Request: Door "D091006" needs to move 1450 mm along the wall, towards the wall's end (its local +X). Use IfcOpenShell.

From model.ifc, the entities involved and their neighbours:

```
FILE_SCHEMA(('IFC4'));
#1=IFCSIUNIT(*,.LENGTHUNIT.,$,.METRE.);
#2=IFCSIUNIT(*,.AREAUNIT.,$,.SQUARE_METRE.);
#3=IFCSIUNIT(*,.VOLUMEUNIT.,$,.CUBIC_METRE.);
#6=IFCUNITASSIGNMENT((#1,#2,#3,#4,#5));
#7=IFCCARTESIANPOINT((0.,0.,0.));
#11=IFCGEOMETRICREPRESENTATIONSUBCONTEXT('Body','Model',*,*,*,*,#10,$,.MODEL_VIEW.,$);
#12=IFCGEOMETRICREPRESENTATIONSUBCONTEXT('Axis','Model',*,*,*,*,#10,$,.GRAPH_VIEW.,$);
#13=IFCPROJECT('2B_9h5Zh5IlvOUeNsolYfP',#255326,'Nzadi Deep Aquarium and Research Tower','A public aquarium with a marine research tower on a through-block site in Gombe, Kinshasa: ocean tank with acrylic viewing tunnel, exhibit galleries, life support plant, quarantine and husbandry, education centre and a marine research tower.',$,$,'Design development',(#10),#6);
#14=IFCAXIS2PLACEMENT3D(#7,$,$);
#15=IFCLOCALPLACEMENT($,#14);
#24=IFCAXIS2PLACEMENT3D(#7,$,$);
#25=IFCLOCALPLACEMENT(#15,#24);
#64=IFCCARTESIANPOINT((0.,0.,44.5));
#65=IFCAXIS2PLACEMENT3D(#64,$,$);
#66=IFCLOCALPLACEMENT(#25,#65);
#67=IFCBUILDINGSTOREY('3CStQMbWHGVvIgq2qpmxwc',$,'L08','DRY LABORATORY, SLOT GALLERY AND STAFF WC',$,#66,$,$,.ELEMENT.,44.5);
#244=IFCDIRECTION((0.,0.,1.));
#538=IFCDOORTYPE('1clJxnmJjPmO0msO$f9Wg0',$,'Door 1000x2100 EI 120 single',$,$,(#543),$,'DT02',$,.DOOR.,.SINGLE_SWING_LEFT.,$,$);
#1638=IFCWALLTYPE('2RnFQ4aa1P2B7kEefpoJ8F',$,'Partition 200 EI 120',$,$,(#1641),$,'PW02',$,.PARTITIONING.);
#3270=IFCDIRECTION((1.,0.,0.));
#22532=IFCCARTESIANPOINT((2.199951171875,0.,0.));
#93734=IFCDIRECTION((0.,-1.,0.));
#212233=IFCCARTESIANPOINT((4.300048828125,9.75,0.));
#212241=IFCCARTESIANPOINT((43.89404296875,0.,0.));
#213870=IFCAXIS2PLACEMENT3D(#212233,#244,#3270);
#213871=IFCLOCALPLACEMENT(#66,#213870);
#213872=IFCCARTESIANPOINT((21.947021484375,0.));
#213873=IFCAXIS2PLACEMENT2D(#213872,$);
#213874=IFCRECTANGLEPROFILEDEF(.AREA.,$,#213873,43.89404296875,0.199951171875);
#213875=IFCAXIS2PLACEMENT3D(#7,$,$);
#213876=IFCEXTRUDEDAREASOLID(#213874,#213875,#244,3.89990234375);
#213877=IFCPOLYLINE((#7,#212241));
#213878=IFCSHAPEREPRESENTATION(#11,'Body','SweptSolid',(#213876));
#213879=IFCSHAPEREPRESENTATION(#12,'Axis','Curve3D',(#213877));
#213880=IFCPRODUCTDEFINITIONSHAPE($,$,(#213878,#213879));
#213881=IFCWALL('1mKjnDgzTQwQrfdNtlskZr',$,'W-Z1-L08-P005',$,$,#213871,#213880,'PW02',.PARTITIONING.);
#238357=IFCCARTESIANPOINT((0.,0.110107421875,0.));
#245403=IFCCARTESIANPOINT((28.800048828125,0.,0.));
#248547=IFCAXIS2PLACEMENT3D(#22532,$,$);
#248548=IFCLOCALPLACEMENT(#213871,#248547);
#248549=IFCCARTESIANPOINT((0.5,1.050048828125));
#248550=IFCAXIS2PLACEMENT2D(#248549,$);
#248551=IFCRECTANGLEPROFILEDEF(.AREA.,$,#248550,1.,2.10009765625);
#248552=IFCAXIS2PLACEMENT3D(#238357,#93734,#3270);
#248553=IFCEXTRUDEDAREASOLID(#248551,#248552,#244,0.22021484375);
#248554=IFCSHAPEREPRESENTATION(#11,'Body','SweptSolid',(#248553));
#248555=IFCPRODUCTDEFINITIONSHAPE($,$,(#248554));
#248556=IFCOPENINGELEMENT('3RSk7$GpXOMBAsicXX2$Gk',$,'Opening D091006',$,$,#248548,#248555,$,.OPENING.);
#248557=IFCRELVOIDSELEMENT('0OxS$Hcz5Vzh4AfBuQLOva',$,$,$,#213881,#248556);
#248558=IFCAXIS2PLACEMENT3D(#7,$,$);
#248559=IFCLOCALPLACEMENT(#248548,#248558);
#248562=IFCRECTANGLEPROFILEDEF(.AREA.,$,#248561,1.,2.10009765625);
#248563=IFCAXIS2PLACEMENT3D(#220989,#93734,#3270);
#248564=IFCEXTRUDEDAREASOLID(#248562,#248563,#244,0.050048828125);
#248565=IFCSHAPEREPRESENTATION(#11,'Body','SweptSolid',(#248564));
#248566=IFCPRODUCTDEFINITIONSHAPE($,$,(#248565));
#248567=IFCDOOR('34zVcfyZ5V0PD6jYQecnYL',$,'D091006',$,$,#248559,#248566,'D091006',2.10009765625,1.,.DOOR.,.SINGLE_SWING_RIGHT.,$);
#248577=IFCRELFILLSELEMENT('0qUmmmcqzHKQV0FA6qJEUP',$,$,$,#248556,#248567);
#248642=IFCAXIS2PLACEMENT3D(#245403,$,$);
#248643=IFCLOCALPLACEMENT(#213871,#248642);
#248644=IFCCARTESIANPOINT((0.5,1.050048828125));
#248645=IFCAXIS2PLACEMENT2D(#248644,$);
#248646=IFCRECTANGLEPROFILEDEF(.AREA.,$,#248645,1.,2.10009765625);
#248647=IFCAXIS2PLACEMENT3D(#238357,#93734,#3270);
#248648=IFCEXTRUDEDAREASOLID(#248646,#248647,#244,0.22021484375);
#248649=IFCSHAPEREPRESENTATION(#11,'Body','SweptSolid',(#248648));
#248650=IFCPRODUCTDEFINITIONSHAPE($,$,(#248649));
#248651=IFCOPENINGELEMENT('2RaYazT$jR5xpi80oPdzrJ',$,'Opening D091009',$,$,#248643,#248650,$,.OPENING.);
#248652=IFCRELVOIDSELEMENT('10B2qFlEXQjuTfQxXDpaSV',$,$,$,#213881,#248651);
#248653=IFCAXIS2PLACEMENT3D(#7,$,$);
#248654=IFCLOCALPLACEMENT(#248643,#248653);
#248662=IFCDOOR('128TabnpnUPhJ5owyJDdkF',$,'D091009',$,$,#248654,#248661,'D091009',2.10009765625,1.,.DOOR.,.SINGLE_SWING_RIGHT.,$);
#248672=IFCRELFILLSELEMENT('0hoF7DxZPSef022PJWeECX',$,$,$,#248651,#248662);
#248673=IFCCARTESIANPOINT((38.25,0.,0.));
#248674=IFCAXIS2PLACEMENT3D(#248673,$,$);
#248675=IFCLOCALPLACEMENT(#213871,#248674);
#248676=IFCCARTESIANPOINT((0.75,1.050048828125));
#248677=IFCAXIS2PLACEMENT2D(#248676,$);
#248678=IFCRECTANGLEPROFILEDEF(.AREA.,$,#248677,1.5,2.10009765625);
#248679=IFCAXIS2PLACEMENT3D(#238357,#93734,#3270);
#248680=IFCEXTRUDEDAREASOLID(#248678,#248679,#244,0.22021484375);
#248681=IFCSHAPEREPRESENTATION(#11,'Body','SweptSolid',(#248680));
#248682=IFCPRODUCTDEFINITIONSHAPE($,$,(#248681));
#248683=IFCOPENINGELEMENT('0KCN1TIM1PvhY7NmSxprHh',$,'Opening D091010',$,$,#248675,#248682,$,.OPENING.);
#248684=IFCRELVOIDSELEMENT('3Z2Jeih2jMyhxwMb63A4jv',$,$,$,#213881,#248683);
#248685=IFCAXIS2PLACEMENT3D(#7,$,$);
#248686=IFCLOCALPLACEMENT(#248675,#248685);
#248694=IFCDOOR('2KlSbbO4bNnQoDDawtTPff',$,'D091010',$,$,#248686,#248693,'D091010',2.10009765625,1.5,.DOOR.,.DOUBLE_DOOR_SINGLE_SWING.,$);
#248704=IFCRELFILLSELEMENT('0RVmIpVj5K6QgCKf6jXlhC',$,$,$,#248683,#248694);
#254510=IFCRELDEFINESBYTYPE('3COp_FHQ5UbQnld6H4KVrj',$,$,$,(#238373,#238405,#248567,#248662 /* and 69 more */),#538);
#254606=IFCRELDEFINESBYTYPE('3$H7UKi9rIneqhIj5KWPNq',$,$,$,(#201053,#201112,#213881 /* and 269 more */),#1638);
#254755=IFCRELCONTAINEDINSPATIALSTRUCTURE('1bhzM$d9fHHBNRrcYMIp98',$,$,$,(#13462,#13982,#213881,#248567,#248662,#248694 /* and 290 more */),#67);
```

```python
import ifcopenshell
import ifcopenshell.api.geometry
import ifcopenshell.util.placement
import ifcopenshell.util.unit

model = ifcopenshell.open("model.ifc")
unit_scale = ifcopenshell.util.unit.calculate_unit_scale(model)

door = model.by_guid("34zVcfyZ5V0PD6jYQecnYL")
opening = door.FillsVoids[0].RelatingOpeningElement
wall = opening.VoidsElements[0].RelatingBuildingElement

wall_matrix = ifcopenshell.util.placement.get_local_placement(wall.ObjectPlacement)
shift = wall_matrix[:3, 0] * 1.45 / unit_scale
before = ifcopenshell.util.placement.get_local_placement(door.ObjectPlacement)[:3, 3].copy()

# The door is placed relative to its opening, so it follows when the opening moves.
matrix = ifcopenshell.util.placement.get_local_placement(opening.ObjectPlacement)
matrix[:3, 3] += shift
ifcopenshell.api.geometry.edit_object_placement(
    model, product=opening, matrix=matrix, is_si=False, should_transform_children=True
)

after = ifcopenshell.util.placement.get_local_placement(door.ObjectPlacement)[:3, 3]
print("door moved by", (after - before).round(3) + 0.0)

model.write("model_updated.ifc")
```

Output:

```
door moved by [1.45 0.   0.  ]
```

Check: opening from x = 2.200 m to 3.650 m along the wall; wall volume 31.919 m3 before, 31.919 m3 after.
